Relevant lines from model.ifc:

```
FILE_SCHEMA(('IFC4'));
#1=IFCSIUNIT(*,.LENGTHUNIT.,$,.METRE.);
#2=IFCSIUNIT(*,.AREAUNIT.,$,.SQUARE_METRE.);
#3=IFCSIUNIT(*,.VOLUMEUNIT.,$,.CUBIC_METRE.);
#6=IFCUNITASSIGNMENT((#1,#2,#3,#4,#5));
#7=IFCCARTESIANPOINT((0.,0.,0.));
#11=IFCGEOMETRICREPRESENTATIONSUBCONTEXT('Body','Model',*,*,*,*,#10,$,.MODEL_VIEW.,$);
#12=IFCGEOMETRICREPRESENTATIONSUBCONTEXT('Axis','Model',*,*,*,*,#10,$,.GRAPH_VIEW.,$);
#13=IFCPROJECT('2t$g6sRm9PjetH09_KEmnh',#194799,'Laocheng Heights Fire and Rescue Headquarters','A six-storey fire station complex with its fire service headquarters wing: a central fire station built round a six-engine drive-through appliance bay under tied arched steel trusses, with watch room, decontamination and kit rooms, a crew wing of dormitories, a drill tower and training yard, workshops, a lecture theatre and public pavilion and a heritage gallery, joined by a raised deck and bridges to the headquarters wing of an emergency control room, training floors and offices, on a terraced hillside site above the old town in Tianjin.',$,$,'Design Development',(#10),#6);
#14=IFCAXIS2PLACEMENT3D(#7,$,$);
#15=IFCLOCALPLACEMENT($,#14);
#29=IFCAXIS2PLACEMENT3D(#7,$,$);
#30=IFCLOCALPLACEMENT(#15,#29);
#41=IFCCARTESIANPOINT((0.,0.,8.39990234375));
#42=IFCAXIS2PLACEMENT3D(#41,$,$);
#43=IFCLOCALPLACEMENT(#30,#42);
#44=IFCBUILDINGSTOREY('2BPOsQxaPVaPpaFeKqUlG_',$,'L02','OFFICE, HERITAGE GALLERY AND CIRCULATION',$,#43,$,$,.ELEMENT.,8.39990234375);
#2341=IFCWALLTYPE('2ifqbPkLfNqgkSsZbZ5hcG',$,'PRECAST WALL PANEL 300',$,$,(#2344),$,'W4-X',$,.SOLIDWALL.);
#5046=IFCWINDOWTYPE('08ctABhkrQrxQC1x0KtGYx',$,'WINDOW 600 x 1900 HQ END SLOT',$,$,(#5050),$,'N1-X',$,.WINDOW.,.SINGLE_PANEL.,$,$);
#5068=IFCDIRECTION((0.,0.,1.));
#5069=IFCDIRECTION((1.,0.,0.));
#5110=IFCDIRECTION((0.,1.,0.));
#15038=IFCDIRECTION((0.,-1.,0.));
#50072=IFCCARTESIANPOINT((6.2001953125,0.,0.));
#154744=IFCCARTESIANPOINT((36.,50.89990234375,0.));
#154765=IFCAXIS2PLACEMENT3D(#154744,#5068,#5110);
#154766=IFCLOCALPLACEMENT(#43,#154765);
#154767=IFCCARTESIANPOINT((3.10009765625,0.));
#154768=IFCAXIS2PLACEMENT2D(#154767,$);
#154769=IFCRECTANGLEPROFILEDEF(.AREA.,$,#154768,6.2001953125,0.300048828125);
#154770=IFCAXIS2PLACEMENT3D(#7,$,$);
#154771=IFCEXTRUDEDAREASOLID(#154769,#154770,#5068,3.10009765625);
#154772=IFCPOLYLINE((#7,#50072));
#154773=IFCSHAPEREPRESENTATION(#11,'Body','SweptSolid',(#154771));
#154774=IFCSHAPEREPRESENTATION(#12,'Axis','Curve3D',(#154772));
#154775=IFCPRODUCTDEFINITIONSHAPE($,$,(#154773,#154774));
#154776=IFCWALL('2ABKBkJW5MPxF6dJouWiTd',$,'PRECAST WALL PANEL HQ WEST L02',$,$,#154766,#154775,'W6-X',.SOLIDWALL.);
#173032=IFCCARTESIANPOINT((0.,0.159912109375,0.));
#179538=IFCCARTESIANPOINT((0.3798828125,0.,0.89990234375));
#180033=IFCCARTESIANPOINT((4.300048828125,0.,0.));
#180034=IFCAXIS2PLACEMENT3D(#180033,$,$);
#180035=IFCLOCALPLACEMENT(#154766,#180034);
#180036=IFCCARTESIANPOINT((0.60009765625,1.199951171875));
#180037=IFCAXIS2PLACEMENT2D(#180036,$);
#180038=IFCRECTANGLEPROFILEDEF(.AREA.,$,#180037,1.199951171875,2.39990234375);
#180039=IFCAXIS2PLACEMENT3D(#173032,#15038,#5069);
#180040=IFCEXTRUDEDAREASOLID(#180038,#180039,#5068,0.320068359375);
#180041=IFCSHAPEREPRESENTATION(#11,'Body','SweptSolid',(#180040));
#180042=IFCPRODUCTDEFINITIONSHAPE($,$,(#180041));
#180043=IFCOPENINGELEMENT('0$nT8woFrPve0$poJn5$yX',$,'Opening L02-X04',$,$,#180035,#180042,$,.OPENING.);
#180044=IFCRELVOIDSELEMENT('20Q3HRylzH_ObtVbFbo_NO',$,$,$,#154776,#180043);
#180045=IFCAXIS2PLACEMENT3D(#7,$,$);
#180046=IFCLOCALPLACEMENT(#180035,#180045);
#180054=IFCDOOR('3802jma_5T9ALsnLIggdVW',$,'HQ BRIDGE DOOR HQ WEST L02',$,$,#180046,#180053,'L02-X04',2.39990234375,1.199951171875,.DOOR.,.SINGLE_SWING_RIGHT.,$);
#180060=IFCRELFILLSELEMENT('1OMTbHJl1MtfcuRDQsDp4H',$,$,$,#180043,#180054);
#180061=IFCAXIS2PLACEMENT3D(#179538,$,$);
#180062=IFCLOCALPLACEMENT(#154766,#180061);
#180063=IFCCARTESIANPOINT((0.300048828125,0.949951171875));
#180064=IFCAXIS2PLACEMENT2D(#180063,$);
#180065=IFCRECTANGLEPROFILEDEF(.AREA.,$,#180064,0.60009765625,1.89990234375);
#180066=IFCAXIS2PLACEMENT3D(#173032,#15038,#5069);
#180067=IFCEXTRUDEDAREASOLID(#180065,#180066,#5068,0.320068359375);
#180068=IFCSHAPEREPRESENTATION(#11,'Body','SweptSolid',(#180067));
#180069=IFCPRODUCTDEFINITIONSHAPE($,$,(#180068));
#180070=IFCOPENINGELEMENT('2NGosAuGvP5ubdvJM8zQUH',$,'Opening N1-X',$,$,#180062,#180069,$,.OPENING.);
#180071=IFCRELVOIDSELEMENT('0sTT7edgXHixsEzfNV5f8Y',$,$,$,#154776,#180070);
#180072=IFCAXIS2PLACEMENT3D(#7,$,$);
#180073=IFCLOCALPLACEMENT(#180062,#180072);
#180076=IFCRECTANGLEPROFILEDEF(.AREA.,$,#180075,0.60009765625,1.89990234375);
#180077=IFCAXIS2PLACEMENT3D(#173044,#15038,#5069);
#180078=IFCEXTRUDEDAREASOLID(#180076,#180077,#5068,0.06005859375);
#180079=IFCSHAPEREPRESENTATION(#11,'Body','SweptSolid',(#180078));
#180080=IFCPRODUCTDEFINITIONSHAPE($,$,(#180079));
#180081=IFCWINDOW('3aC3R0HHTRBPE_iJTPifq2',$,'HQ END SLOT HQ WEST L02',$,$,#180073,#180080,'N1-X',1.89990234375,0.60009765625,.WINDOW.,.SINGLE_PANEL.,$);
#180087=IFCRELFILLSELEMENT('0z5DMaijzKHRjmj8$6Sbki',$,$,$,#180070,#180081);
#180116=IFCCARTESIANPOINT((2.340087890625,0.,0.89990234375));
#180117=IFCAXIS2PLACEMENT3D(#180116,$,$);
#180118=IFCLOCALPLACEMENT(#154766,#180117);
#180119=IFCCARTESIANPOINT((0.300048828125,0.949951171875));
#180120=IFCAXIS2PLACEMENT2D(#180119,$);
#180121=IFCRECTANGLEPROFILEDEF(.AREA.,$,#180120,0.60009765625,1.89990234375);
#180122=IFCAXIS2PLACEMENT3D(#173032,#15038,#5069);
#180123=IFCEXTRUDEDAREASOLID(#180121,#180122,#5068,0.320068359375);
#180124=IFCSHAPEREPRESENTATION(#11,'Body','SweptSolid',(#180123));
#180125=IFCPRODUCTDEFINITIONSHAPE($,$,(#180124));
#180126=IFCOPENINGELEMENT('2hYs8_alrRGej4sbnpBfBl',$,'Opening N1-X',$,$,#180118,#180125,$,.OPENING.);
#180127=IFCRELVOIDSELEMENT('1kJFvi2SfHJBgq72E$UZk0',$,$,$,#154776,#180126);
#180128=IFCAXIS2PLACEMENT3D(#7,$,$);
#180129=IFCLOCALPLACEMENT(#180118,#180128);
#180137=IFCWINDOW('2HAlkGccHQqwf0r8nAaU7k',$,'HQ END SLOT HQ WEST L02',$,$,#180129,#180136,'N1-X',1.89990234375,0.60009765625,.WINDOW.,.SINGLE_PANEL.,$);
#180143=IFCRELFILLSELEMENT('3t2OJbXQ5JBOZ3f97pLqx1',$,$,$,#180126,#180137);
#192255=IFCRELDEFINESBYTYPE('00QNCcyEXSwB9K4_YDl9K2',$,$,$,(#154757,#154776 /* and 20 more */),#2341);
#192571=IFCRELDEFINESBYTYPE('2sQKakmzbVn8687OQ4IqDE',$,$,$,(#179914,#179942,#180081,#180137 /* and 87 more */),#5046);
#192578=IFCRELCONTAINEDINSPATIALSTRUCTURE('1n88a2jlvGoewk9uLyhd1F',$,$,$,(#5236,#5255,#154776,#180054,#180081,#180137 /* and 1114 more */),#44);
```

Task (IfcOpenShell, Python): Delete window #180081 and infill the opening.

```python
import ifcopenshell
import ifcopenshell.api.feature
import ifcopenshell.api.root
import ifcopenshell.geom
import ifcopenshell.util.shape

model = ifcopenshell.open("model.ifc")
settings = ifcopenshell.geom.settings()


def volume(element):
    """Net volume in cubic metres, openings subtracted."""
    shape = ifcopenshell.geom.create_shape(settings, element)
    return ifcopenshell.util.shape.get_volume(shape.geometry)


window = model.by_id(180081)
opening = window.FillsVoids[0].RelatingOpeningElement
wall = opening.VoidsElements[0].RelatingBuildingElement
before = volume(wall)

ifcopenshell.api.root.remove_product(model, product=window)
ifcopenshell.api.feature.remove_feature(model, feature=opening)

after = volume(wall)

print(f"wall volume {before:.3f} -> {after:.3f} m3")

model.write("model-out.ifc")
```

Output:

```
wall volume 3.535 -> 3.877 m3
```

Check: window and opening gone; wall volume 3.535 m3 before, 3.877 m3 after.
